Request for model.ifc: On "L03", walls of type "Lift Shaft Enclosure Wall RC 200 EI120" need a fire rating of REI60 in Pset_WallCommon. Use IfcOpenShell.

First a look at what the model holds.

```python
import ifcopenshell
import ifcopenshell.util.element

model = ifcopenshell.open("model.ifc")
print(model.schema)
storey = next(s for s in model.by_type("IfcBuildingStorey") if s.Name == "L03")
walls = [e for e in ifcopenshell.util.element.get_decomposition(storey) if e.is_a("IfcWall")]
seen = {}
for e in walls:
    element_type = ifcopenshell.util.element.get_type(e)
    key = (element_type.Name if element_type != e and element_type else None, ifcopenshell.util.element.get_pset(e, "Pset_WallCommon", "FireRating"))
    seen[key] = seen.get(key, 0) + 1
for (name, value), count in sorted(seen.items(), key=str):
    print(count, "x", name, "|", value)
```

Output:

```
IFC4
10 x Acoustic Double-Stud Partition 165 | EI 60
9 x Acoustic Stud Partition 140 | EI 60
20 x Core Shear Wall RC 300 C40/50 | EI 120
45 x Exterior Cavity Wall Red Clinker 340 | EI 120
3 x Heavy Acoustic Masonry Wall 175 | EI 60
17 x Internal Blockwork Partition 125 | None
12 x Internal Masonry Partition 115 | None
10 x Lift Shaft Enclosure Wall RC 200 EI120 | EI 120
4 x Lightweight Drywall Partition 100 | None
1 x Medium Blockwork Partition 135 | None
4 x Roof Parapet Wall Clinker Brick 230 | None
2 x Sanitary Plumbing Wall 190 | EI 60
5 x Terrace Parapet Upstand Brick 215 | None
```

```python
import ifcopenshell
import ifcopenshell.api.pset
import ifcopenshell.util.element

model = ifcopenshell.open("model.ifc")

storey = next(s for s in model.by_type("IfcBuildingStorey") if s.Name == "L03")
walls = [e for e in ifcopenshell.util.element.get_decomposition(storey) if e.is_a("IfcWall")]

count = 0
for e in walls:
    element_type = ifcopenshell.util.element.get_type(e)
    if element_type in (None, e) or element_type.Name != "Lift Shaft Enclosure Wall RC 200 EI120":
        continue
    # add_pset returns the element's existing set when there is one.
    pset = ifcopenshell.api.pset.add_pset(model, product=e, name="Pset_WallCommon")
    ifcopenshell.api.pset.edit_pset(model, pset=pset, properties={"FireRating": "REI60"})
    count += 1

print(count, "walls updated")

model.write("model_updated.ifc")
```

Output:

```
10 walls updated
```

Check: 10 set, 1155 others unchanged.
